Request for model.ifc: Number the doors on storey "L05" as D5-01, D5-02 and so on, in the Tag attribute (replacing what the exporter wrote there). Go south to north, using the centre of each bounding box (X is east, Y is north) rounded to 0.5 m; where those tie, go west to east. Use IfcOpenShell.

First a look at what the model holds.

```python
import ifcopenshell
import ifcopenshell.util.element
import ifcopenshell.util.placement

model = ifcopenshell.open("model.ifc")
print(model.schema)
storey = next(s for s in model.by_type("IfcBuildingStorey") if s.Name == "L05")
doors = [e for e in ifcopenshell.util.element.get_decomposition(storey) if e.is_a("IfcDoor")]
for e in sorted(doors, key=lambda e: e.id()):
    origin = ifcopenshell.util.placement.get_local_placement(e.ObjectPlacement)[:3, 3]
    print(e.id(), e.Tag, e.Name, origin.round(2) + 0.0, sep=" | ")
```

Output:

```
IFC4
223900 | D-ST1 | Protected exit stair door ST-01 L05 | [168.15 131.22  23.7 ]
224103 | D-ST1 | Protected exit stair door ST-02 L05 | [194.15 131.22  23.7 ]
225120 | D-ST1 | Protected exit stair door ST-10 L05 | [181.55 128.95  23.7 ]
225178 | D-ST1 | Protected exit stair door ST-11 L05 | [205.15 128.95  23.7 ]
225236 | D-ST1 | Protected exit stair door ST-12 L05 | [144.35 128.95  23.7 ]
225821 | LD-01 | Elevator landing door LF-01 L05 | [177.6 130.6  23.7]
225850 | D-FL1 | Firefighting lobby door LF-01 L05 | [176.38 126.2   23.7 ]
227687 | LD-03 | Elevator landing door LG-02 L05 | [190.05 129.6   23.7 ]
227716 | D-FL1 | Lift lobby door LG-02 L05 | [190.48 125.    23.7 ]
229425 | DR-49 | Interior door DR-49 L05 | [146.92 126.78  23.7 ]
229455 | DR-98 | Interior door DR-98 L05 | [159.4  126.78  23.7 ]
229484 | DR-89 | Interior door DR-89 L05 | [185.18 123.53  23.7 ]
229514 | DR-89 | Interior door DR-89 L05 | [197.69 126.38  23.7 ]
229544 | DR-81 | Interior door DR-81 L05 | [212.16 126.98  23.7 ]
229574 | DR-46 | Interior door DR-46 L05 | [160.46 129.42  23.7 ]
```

```python
import ifcopenshell
import ifcopenshell.geom
import ifcopenshell.util.element
import ifcopenshell.util.shape

model = ifcopenshell.open("model.ifc")
settings = ifcopenshell.geom.settings()
settings.set("use-world-coords", True)


def centre(element):
    shape = ifcopenshell.geom.create_shape(settings, element)
    return ifcopenshell.util.shape.get_bbox_centroid(shape.geometry)


storey = next(s for s in model.by_type("IfcBuildingStorey") if s.Name == "L05")
doors = [e for e in ifcopenshell.util.element.get_decomposition(storey) if e.is_a("IfcDoor")]

# Insertion points can sit at a corner or the storey origin, so sort by the geometry (in metres).
centres = {e: centre(e) for e in doors}
doors.sort(key=lambda e: (round(centres[e][1] / 0.5), centres[e][0]))

for i, e in enumerate(doors, start=1):
    number = f"D5-{i:02d}"
    e.Tag = number
    print(e.id(), number)

model.write("model-out.ifc")
```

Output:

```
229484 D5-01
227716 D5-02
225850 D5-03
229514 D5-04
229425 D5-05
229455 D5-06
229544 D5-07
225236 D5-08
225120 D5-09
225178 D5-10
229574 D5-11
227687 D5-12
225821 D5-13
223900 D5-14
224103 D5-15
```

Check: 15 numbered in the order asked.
